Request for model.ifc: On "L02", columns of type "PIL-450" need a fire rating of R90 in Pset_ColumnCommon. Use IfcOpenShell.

First a look at what the model holds.

```python
import ifcopenshell
import ifcopenshell.util.element

model = ifcopenshell.open("model.ifc")
print(model.schema)
storey = next(s for s in model.by_type("IfcBuildingStorey") if s.Name == "L02")
columns = [e for e in ifcopenshell.util.element.get_decomposition(storey) if e.is_a("IfcColumn")]
seen = {}
for e in columns:
    element_type = ifcopenshell.util.element.get_type(e)
    key = (element_type.Name if element_type != e and element_type else None, ifcopenshell.util.element.get_pset(e, "Pset_ColumnCommon", "FireRating"))
    seen[key] = seen.get(key, 0) + 1
for (name, value), count in sorted(seen.items(), key=str):
    print(count, "x", name, "|", value)
```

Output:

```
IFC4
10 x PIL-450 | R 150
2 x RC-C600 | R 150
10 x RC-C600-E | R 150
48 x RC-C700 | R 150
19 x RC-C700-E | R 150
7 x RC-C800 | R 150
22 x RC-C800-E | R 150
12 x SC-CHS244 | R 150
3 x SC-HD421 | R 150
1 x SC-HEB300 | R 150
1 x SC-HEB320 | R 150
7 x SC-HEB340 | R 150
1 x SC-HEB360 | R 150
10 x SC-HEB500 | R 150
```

```python
import ifcopenshell
import ifcopenshell.api.pset
import ifcopenshell.util.element

model = ifcopenshell.open("model.ifc")

storey = next(s for s in model.by_type("IfcBuildingStorey") if s.Name == "L02")
columns = [e for e in ifcopenshell.util.element.get_decomposition(storey) if e.is_a("IfcColumn")]

count = 0
for e in columns:
    element_type = ifcopenshell.util.element.get_type(e)
    if element_type in (None, e) or element_type.Name != "PIL-450":
        continue
    # add_pset returns the element's existing set when there is one.
    pset = ifcopenshell.api.pset.add_pset(model, product=e, name="Pset_ColumnCommon")
    ifcopenshell.api.pset.edit_pset(model, pset=pset, properties={"FireRating": "R90"})
    count += 1

print(count, "columns updated")

model.write("model-out.ifc")
```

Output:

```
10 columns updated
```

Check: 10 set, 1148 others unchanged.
